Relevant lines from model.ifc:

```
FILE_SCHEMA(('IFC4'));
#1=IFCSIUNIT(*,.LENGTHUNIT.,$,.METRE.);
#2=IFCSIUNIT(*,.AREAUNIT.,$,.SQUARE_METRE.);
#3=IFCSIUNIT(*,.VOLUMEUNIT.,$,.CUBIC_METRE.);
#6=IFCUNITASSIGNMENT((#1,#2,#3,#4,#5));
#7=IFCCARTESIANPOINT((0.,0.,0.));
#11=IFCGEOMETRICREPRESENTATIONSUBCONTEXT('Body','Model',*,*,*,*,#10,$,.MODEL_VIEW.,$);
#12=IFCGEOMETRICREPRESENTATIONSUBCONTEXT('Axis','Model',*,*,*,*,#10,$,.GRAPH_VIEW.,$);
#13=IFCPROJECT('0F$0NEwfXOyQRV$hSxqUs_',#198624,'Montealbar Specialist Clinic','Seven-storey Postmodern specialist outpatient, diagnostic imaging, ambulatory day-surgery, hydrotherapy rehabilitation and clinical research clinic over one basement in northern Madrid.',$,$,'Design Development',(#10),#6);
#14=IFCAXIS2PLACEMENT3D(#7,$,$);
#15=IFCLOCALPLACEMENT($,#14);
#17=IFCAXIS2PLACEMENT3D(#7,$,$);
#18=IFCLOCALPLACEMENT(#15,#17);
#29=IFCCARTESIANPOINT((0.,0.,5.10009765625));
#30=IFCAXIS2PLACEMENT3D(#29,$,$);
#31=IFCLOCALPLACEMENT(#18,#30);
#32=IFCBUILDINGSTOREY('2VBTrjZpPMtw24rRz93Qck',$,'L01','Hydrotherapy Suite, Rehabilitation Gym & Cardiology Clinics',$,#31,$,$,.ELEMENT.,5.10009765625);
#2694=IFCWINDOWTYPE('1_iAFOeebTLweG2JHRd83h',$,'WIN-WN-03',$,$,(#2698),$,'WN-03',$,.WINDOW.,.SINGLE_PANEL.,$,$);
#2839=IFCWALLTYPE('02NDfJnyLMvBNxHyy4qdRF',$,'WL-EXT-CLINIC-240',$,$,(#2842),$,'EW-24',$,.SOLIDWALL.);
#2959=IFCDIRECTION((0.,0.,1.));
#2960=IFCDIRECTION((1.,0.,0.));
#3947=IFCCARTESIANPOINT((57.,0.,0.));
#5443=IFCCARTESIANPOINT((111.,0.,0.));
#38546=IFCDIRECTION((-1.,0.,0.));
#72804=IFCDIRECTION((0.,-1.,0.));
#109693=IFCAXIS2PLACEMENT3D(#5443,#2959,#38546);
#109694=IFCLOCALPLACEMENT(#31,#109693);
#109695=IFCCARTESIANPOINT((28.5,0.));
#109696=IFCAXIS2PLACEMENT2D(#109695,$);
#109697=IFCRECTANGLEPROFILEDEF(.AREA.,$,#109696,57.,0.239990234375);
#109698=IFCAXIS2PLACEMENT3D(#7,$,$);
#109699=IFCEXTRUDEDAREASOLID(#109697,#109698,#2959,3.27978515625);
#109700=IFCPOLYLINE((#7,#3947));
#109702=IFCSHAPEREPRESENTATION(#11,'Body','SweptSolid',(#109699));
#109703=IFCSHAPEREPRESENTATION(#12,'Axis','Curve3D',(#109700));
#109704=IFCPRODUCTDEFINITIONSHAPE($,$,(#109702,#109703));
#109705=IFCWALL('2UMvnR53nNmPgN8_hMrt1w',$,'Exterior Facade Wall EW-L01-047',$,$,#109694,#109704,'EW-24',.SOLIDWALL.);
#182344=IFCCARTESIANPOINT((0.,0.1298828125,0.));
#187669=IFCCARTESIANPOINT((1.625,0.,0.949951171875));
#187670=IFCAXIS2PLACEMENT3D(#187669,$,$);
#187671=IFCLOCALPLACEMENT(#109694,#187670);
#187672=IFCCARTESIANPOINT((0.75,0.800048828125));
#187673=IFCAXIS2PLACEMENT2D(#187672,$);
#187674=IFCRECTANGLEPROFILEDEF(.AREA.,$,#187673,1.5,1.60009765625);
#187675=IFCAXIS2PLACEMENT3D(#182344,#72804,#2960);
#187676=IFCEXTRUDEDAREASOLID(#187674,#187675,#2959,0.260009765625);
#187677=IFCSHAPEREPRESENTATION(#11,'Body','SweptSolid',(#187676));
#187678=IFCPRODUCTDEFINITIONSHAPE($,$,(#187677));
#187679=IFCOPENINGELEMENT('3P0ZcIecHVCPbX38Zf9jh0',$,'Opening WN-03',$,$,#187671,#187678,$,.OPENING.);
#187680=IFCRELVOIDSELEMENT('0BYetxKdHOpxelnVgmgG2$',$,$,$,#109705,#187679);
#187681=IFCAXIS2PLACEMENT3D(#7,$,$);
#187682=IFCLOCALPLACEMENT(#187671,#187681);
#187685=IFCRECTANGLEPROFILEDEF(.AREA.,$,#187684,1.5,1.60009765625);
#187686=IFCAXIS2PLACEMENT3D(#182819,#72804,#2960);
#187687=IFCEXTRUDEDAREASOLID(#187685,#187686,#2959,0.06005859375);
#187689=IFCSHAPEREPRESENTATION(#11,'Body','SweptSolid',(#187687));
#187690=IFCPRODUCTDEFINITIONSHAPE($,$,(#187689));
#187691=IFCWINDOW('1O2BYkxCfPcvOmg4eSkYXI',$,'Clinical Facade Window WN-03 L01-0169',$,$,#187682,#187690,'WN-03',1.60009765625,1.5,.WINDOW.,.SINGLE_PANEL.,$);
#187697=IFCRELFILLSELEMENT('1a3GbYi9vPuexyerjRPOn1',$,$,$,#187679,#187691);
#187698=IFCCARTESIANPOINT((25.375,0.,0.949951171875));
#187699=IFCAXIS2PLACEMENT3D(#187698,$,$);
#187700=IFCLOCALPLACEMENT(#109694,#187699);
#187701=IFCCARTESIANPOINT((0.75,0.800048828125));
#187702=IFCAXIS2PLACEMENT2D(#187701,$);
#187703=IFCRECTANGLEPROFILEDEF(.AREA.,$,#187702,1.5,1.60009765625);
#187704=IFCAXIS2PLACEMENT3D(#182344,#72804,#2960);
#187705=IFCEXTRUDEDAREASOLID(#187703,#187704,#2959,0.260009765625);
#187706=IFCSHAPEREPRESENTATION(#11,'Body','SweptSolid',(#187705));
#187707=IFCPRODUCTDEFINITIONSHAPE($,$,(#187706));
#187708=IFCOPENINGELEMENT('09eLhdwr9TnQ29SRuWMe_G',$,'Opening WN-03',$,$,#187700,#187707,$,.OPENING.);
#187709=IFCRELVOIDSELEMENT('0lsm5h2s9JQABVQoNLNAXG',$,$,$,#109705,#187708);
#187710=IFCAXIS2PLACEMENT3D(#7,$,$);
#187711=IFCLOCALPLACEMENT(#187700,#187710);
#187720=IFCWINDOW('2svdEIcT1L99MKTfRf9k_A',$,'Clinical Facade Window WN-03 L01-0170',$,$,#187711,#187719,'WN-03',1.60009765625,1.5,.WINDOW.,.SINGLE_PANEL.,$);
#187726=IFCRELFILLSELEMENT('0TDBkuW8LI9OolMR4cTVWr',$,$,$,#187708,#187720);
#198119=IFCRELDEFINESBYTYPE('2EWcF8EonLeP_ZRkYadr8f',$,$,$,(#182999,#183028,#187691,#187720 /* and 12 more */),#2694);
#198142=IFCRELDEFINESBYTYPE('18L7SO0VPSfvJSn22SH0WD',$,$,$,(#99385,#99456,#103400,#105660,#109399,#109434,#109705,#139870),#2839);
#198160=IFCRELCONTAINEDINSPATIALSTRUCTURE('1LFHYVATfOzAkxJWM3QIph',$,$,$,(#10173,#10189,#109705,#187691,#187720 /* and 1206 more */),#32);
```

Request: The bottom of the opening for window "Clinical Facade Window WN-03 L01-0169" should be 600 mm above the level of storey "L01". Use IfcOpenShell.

```python
import numpy as np
import ifcopenshell
import ifcopenshell.api.geometry
import ifcopenshell.geom
import ifcopenshell.util.element
import ifcopenshell.util.placement
import ifcopenshell.util.shape
import ifcopenshell.util.unit

model = ifcopenshell.open("model.ifc")
unit_scale = ifcopenshell.util.unit.calculate_unit_scale(model)

window = model.by_guid("1O2BYkxCfPcvOmg4eSkYXI")
opening = window.FillsVoids[0].RelatingOpeningElement
storey = ifcopenshell.util.element.get_container(window, ifc_class="IfcBuildingStorey")
level = ifcopenshell.util.placement.get_local_placement(storey.ObjectPlacement)[2, 3]

# The opening's origin need not be at the sill, so measure its lowest point.
shape = ifcopenshell.geom.create_shape(ifcopenshell.geom.settings(), opening)
bottom = ifcopenshell.util.shape.get_shape_bottom_elevation(shape, shape.geometry) / unit_scale
dz = level + 0.6 / unit_scale - bottom

shift = np.array([0.0, 0.0, dz])
# The window is placed relative to its opening, so it follows when the opening moves.
matrix = ifcopenshell.util.placement.get_local_placement(opening.ObjectPlacement)
matrix[:3, 3] += shift
ifcopenshell.api.geometry.edit_object_placement(
    model, product=opening, matrix=matrix, is_si=False, should_transform_children=True
)

print(f"moved by {dz * unit_scale:+.3f} m")

model.write("model-out.ifc")
```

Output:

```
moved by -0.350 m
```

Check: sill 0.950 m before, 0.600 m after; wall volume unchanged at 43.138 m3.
